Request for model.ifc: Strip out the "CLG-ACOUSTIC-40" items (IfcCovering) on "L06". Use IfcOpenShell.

First a look at what the model holds.

```python
import ifcopenshell
import ifcopenshell.util.element

model = ifcopenshell.open("model.ifc")
print(model.schema)
storey = next(s for s in model.by_type("IfcBuildingStorey") if s.Name == "L06")
coverings = [e for e in ifcopenshell.util.element.get_decomposition(storey) if e.is_a("IfcCovering")]
seen = {}
for e in coverings:
    element_type = ifcopenshell.util.element.get_type(e)
    name = element_type.Name if element_type not in (None, e) else None
    seen[name] = seen.get(name, 0) + 1
for name, count in sorted(seen.items(), key=str):
    print(count, "x", name)
```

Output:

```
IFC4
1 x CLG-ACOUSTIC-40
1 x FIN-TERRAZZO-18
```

```python
import ifcopenshell
import ifcopenshell.api.root
import ifcopenshell.util.element

model = ifcopenshell.open("model.ifc")

storey = next(s for s in model.by_type("IfcBuildingStorey") if s.Name == "L06")
coverings = [e for e in ifcopenshell.util.element.get_decomposition(storey) if e.is_a("IfcCovering")]
targets = [e for e in coverings if (t := ifcopenshell.util.element.get_type(e)) not in (None, e) and t.Name == "CLG-ACOUSTIC-40"]

for e in targets:
    ifcopenshell.api.root.remove_product(model, product=e)
print(len(targets), "removed")

model.write("model_edited.ifc")
```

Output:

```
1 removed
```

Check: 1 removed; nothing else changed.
